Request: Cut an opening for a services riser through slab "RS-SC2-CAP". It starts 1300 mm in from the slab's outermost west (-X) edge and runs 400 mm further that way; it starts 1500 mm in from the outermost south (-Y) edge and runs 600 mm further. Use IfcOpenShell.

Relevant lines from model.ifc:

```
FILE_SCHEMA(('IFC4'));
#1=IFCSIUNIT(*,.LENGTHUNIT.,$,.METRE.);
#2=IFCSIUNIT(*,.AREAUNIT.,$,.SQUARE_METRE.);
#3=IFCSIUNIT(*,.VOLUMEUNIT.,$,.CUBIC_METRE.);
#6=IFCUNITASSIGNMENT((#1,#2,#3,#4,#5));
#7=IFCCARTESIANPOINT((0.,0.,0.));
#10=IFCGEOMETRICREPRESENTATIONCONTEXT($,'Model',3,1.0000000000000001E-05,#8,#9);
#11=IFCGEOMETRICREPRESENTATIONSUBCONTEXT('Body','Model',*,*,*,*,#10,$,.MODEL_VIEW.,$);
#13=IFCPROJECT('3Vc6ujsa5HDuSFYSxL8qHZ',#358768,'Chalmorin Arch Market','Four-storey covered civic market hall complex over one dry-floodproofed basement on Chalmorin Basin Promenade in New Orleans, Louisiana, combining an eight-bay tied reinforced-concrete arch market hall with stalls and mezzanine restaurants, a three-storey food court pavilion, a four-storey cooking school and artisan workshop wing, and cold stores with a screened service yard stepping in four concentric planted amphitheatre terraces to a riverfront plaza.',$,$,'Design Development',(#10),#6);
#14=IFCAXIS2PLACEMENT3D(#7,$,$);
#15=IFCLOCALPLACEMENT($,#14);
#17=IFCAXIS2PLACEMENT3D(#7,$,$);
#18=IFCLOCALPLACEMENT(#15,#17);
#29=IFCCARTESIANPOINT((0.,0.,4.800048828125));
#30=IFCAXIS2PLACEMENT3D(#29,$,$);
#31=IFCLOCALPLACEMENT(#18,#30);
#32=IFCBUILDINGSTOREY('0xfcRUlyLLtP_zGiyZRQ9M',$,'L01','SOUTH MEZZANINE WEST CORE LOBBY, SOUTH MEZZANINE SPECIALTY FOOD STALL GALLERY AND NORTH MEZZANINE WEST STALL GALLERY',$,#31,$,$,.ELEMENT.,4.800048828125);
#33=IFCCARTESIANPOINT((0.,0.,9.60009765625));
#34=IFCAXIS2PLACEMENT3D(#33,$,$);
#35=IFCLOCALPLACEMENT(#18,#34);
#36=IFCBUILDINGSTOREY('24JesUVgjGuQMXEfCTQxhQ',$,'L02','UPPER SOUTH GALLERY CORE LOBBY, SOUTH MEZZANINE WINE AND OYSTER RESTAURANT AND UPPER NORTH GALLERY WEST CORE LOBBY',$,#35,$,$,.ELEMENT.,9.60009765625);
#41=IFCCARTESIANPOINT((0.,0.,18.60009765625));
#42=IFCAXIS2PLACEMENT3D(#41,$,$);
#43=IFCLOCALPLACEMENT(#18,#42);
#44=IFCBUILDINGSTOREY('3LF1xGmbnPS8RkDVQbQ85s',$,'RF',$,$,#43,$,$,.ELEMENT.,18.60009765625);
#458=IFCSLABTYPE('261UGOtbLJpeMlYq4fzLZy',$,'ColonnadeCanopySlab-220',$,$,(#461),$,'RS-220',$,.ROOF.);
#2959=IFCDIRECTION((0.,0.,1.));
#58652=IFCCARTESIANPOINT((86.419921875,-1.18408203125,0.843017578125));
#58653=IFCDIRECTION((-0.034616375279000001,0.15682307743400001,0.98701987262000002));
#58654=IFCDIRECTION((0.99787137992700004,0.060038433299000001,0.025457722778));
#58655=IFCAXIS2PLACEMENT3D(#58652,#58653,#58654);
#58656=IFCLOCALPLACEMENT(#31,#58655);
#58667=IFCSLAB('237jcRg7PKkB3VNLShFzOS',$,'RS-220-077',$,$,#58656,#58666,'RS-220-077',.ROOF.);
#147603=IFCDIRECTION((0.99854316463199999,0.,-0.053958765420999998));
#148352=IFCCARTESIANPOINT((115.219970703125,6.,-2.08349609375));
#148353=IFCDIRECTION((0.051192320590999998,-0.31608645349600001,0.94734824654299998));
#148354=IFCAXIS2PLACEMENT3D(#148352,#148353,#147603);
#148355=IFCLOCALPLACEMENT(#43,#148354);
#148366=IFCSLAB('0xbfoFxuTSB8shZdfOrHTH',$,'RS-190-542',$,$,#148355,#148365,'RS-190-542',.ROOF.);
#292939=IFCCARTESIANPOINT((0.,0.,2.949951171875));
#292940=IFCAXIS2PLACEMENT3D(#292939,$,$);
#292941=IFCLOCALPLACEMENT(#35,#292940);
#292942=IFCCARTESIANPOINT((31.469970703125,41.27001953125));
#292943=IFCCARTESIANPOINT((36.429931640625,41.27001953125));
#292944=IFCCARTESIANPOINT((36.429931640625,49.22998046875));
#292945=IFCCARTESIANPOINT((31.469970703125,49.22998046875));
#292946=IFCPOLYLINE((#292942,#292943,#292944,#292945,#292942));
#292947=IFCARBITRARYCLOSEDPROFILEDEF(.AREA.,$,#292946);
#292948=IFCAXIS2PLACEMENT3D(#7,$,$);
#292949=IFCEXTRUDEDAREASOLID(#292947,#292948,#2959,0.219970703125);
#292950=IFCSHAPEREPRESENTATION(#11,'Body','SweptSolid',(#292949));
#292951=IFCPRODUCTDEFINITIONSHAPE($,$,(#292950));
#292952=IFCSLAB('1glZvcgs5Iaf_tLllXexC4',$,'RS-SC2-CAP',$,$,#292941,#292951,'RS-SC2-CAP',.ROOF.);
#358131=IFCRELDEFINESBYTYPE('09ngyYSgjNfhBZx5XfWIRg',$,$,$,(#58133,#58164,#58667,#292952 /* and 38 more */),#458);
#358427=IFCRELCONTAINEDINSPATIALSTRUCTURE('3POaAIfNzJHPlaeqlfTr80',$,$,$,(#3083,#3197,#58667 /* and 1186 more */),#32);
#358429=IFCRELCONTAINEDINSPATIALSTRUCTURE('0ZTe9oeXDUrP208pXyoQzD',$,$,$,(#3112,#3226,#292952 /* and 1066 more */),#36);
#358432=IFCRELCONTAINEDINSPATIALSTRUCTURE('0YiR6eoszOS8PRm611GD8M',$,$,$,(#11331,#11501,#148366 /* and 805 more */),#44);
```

```python
import numpy as np
import ifcopenshell
import ifcopenshell.api.feature
import ifcopenshell.api.geometry
import ifcopenshell.api.root
import ifcopenshell.geom
import ifcopenshell.util.placement
import ifcopenshell.util.representation
import ifcopenshell.util.shape
import ifcopenshell.util.unit

model = ifcopenshell.open("model.ifc")
unit_scale = ifcopenshell.util.unit.calculate_unit_scale(model)
settings = ifcopenshell.geom.settings()


def volume(element):
    """Net volume in cubic metres, openings subtracted."""
    shape = ifcopenshell.geom.create_shape(settings, element)
    return ifcopenshell.util.shape.get_volume(shape.geometry)


slab = model.by_guid("1glZvcgs5Iaf_tLllXexC4")
before = volume(slab)

# Extent in the slab's own axes, in metres. The edges named are its -X and -Y sides.
slab_shape = ifcopenshell.geom.create_shape(settings, slab)
vertices = ifcopenshell.util.shape.get_vertices(slab_shape.geometry)
x_min, y_min, bottom = vertices.min(axis=0)
top = vertices[:, 2].max()

opening = ifcopenshell.api.root.create_entity(model, ifc_class="IfcOpeningElement", name="Services riser opening", predefined_type="OPENING")
context = ifcopenshell.util.representation.get_context(model, "Model", "Body", "MODEL_VIEW")
width, depth = 0.4, 0.6
outline = [(0.0, 0.0), (width, 0.0), (width, depth), (0.0, depth), (0.0, 0.0)]
# Overshoot both faces by 50 mm so the cut is clean.
shape = ifcopenshell.api.geometry.add_slab_representation(
    model, context=context, depth=top - bottom + 0.1, polyline=outline
)
ifcopenshell.api.geometry.assign_representation(model, product=opening, representation=shape)

matrix = ifcopenshell.util.placement.get_local_placement(slab.ObjectPlacement)
matrix[:, 3] = matrix @ np.append(np.array([x_min + 1.3, y_min + 1.5, bottom - 0.05]) / unit_scale, 1.0)
ifcopenshell.api.geometry.edit_object_placement(model, product=opening, matrix=matrix, is_si=False)
ifcopenshell.api.feature.add_feature(model, feature=opening, element=slab)

after = volume(slab)

print(f"slab volume {before:.3f} -> {after:.3f} m3")

model.write("model-out.ifc")
```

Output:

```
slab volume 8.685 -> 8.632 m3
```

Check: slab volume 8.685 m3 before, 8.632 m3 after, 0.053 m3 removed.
